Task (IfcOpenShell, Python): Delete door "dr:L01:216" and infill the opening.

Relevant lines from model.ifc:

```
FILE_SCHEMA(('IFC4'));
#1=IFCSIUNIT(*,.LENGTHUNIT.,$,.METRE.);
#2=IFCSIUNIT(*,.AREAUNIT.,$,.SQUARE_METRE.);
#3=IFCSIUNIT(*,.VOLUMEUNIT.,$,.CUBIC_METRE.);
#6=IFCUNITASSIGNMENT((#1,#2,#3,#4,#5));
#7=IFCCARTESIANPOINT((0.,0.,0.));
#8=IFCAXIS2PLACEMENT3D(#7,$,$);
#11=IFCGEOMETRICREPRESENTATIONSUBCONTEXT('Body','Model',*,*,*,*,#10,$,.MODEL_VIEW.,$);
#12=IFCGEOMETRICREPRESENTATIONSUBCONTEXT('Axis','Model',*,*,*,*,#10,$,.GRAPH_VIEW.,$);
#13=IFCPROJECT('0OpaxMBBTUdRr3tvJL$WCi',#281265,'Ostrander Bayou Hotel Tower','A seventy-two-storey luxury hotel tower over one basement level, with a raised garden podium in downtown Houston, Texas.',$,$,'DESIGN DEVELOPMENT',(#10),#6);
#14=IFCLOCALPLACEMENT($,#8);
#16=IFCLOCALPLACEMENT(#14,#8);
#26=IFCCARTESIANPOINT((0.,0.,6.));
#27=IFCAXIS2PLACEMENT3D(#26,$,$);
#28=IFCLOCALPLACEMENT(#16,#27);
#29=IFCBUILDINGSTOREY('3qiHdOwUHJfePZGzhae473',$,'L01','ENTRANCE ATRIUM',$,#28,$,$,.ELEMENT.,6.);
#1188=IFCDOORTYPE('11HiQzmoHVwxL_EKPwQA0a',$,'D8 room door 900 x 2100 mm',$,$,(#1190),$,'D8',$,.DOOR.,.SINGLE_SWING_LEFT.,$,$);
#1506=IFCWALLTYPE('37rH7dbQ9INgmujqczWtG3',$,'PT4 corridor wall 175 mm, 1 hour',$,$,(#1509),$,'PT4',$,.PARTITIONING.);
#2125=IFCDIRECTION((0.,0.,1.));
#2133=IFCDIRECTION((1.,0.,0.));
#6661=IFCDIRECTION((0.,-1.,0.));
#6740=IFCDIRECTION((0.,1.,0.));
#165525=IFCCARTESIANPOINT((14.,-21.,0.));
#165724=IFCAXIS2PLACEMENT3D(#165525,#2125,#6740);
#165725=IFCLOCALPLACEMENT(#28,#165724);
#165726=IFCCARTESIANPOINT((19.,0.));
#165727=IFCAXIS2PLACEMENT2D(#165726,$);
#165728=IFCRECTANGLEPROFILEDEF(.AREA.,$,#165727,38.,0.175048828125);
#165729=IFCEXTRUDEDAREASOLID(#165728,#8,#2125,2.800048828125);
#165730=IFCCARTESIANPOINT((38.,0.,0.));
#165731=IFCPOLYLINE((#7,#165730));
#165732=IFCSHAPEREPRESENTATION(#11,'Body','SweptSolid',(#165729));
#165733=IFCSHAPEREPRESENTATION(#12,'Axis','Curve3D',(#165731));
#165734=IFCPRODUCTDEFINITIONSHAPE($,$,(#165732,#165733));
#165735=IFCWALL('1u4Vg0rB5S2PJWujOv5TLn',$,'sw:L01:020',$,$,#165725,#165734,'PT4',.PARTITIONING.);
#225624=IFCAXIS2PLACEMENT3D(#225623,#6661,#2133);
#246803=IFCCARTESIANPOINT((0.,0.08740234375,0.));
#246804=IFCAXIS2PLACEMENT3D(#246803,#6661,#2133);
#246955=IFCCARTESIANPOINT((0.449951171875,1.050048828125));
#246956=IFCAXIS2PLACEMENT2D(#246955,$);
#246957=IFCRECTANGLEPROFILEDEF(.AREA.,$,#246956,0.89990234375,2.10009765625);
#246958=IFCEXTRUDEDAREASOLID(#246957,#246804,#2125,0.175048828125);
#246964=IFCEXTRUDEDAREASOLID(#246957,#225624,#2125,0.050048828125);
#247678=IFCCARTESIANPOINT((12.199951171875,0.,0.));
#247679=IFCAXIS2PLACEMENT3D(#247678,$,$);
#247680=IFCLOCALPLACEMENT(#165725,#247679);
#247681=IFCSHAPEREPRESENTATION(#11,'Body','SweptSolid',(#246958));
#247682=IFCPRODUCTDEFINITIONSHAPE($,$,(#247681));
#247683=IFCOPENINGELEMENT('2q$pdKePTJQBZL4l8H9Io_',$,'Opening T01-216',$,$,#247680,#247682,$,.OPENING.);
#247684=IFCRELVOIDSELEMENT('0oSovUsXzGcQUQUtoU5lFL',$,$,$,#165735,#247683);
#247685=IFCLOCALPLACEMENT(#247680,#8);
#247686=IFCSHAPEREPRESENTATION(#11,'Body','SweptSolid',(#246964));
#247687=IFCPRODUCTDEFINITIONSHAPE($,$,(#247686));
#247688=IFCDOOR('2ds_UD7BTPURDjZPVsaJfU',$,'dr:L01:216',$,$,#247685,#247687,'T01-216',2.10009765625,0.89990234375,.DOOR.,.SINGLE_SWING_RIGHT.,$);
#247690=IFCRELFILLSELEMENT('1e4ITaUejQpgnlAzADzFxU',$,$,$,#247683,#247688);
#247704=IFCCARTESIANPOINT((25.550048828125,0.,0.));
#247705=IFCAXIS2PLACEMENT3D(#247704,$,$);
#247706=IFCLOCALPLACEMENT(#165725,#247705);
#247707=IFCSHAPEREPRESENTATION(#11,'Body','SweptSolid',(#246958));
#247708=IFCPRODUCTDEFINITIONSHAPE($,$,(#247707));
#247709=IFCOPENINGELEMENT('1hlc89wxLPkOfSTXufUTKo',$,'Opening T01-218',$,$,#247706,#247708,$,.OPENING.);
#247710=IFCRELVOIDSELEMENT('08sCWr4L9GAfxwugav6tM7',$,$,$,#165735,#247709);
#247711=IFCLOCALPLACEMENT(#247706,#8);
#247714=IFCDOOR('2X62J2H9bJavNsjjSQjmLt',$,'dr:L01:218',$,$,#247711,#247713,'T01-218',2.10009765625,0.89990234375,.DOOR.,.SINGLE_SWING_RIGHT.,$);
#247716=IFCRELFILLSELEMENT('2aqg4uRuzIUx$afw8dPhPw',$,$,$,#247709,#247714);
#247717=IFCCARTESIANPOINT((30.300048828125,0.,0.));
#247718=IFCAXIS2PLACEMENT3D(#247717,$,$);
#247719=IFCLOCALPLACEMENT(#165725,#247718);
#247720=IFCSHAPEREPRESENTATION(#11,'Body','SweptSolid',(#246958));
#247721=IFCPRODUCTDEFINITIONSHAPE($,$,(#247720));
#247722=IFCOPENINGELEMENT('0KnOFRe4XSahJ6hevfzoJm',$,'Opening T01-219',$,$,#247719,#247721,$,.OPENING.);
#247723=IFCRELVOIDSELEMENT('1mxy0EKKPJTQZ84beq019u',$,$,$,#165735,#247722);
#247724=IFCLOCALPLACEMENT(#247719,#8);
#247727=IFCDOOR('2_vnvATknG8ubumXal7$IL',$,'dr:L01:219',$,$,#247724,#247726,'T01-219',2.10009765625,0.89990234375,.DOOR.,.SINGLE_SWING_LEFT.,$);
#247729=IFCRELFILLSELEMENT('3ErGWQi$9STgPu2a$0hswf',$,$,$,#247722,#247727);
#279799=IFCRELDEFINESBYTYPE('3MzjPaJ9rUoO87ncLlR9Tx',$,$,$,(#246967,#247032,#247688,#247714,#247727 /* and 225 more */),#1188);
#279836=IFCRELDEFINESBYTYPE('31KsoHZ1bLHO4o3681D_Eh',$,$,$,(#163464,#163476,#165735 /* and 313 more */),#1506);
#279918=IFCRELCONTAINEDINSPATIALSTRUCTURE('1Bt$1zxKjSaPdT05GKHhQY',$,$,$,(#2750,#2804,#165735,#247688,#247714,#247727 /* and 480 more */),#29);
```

```python
import ifcopenshell
import ifcopenshell.api.feature
import ifcopenshell.api.root
import ifcopenshell.geom
import ifcopenshell.util.shape

model = ifcopenshell.open("model.ifc")
settings = ifcopenshell.geom.settings()


def volume(element):
    """Net volume in cubic metres, openings subtracted."""
    shape = ifcopenshell.geom.create_shape(settings, element)
    return ifcopenshell.util.shape.get_volume(shape.geometry)


door = model.by_guid("2ds_UD7BTPURDjZPVsaJfU")
opening = door.FillsVoids[0].RelatingOpeningElement
wall = opening.VoidsElements[0].RelatingBuildingElement
before = volume(wall)

ifcopenshell.api.root.remove_product(model, product=door)
ifcopenshell.api.feature.remove_feature(model, feature=opening)

after = volume(wall)

print(f"wall volume {before:.3f} -> {after:.3f} m3")

model.write("model_updated.ifc")
```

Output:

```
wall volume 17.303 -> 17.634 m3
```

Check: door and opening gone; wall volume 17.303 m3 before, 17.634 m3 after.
